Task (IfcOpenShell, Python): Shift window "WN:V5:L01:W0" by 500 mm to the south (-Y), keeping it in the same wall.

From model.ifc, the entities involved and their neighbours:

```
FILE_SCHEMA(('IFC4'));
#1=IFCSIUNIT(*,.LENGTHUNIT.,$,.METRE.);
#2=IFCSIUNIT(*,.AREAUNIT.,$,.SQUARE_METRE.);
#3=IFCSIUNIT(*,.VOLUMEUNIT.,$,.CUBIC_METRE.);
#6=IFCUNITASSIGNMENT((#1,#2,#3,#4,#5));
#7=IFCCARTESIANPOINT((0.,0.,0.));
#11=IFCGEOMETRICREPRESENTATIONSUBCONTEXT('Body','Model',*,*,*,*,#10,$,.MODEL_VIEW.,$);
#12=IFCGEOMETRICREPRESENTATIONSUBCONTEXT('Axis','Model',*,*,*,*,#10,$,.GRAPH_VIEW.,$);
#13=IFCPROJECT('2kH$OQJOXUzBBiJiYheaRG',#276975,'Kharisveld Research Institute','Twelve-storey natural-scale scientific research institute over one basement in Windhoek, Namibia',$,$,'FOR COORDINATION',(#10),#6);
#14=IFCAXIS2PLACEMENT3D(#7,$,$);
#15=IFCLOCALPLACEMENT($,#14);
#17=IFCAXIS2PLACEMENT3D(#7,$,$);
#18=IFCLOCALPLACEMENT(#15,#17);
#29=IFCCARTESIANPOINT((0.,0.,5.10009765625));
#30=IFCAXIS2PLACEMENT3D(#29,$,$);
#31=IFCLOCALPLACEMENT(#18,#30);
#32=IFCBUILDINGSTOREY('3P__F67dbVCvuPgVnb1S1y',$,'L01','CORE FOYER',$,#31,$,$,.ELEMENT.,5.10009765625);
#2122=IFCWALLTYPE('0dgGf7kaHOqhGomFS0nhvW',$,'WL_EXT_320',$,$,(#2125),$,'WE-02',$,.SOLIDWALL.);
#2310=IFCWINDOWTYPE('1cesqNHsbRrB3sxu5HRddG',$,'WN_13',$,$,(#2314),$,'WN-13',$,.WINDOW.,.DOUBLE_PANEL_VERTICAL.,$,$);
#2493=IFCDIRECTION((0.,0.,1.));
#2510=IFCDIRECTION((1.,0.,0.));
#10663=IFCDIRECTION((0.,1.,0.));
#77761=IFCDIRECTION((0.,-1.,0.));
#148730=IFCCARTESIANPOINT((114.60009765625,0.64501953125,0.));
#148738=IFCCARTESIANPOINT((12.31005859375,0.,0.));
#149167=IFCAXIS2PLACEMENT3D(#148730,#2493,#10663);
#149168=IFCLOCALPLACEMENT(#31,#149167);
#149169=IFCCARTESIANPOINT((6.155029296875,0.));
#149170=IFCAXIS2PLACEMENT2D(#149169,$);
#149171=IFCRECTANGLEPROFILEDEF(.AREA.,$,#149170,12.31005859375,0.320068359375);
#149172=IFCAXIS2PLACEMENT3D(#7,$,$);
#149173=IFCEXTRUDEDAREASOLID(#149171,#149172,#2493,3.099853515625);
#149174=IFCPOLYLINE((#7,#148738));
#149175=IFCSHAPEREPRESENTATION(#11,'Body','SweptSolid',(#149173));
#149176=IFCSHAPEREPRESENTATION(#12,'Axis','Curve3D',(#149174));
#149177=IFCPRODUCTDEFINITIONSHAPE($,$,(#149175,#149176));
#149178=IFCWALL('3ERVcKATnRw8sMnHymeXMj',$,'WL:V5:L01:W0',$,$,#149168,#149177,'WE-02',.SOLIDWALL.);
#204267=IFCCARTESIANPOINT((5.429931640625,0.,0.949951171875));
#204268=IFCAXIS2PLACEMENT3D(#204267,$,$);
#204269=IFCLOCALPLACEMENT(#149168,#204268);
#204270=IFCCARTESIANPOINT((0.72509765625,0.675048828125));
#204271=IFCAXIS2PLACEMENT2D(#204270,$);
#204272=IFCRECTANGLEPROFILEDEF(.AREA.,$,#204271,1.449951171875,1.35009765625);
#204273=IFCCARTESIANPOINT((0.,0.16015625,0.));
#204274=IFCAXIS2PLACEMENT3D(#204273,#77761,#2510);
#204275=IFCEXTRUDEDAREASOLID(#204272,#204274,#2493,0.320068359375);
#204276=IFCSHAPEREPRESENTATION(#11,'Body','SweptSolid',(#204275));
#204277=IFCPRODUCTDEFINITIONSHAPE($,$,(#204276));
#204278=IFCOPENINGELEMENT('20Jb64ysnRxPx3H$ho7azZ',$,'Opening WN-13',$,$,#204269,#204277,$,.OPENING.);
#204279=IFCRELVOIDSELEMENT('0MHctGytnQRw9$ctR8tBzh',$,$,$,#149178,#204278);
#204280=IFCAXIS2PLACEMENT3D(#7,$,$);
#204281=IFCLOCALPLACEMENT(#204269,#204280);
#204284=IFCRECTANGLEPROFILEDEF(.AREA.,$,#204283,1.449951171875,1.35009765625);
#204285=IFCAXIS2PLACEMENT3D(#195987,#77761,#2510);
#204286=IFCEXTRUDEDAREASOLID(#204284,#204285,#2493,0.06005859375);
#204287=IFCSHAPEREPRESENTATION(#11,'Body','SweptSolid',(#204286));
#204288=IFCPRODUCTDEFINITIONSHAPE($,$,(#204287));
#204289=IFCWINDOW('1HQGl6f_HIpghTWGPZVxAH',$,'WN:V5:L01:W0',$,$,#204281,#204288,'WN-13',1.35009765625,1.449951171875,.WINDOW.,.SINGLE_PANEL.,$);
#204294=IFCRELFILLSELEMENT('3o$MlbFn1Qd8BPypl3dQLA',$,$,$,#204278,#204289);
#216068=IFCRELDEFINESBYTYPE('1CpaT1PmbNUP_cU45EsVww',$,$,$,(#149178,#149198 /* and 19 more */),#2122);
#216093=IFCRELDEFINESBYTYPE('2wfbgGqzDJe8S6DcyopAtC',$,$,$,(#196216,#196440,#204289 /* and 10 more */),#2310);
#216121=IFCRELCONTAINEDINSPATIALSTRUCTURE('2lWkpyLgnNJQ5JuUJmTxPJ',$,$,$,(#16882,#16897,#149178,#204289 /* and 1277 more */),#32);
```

```python
import ifcopenshell
import ifcopenshell.api.geometry
import ifcopenshell.util.placement
import ifcopenshell.util.unit

model = ifcopenshell.open("model.ifc")
unit_scale = ifcopenshell.util.unit.calculate_unit_scale(model)

window = model.by_guid("1HQGl6f_HIpghTWGPZVxAH")
opening = window.FillsVoids[0].RelatingOpeningElement
wall = opening.VoidsElements[0].RelatingBuildingElement

wall_matrix = ifcopenshell.util.placement.get_local_placement(wall.ObjectPlacement)
shift = wall_matrix[:3, 0] * -0.5 / unit_scale
before = ifcopenshell.util.placement.get_local_placement(window.ObjectPlacement)[:3, 3].copy()

# The window is placed relative to its opening, so it follows when the opening moves.
matrix = ifcopenshell.util.placement.get_local_placement(opening.ObjectPlacement)
matrix[:3, 3] += shift
ifcopenshell.api.geometry.edit_object_placement(
    model, product=opening, matrix=matrix, is_si=False, should_transform_children=True
)

after = ifcopenshell.util.placement.get_local_placement(window.ObjectPlacement)[:3, 3]
print("window moved by", (after - before).round(3) + 0.0)

model.write("model_v2.ifc")
```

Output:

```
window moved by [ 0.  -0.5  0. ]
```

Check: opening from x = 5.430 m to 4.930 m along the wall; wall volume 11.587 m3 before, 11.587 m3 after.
